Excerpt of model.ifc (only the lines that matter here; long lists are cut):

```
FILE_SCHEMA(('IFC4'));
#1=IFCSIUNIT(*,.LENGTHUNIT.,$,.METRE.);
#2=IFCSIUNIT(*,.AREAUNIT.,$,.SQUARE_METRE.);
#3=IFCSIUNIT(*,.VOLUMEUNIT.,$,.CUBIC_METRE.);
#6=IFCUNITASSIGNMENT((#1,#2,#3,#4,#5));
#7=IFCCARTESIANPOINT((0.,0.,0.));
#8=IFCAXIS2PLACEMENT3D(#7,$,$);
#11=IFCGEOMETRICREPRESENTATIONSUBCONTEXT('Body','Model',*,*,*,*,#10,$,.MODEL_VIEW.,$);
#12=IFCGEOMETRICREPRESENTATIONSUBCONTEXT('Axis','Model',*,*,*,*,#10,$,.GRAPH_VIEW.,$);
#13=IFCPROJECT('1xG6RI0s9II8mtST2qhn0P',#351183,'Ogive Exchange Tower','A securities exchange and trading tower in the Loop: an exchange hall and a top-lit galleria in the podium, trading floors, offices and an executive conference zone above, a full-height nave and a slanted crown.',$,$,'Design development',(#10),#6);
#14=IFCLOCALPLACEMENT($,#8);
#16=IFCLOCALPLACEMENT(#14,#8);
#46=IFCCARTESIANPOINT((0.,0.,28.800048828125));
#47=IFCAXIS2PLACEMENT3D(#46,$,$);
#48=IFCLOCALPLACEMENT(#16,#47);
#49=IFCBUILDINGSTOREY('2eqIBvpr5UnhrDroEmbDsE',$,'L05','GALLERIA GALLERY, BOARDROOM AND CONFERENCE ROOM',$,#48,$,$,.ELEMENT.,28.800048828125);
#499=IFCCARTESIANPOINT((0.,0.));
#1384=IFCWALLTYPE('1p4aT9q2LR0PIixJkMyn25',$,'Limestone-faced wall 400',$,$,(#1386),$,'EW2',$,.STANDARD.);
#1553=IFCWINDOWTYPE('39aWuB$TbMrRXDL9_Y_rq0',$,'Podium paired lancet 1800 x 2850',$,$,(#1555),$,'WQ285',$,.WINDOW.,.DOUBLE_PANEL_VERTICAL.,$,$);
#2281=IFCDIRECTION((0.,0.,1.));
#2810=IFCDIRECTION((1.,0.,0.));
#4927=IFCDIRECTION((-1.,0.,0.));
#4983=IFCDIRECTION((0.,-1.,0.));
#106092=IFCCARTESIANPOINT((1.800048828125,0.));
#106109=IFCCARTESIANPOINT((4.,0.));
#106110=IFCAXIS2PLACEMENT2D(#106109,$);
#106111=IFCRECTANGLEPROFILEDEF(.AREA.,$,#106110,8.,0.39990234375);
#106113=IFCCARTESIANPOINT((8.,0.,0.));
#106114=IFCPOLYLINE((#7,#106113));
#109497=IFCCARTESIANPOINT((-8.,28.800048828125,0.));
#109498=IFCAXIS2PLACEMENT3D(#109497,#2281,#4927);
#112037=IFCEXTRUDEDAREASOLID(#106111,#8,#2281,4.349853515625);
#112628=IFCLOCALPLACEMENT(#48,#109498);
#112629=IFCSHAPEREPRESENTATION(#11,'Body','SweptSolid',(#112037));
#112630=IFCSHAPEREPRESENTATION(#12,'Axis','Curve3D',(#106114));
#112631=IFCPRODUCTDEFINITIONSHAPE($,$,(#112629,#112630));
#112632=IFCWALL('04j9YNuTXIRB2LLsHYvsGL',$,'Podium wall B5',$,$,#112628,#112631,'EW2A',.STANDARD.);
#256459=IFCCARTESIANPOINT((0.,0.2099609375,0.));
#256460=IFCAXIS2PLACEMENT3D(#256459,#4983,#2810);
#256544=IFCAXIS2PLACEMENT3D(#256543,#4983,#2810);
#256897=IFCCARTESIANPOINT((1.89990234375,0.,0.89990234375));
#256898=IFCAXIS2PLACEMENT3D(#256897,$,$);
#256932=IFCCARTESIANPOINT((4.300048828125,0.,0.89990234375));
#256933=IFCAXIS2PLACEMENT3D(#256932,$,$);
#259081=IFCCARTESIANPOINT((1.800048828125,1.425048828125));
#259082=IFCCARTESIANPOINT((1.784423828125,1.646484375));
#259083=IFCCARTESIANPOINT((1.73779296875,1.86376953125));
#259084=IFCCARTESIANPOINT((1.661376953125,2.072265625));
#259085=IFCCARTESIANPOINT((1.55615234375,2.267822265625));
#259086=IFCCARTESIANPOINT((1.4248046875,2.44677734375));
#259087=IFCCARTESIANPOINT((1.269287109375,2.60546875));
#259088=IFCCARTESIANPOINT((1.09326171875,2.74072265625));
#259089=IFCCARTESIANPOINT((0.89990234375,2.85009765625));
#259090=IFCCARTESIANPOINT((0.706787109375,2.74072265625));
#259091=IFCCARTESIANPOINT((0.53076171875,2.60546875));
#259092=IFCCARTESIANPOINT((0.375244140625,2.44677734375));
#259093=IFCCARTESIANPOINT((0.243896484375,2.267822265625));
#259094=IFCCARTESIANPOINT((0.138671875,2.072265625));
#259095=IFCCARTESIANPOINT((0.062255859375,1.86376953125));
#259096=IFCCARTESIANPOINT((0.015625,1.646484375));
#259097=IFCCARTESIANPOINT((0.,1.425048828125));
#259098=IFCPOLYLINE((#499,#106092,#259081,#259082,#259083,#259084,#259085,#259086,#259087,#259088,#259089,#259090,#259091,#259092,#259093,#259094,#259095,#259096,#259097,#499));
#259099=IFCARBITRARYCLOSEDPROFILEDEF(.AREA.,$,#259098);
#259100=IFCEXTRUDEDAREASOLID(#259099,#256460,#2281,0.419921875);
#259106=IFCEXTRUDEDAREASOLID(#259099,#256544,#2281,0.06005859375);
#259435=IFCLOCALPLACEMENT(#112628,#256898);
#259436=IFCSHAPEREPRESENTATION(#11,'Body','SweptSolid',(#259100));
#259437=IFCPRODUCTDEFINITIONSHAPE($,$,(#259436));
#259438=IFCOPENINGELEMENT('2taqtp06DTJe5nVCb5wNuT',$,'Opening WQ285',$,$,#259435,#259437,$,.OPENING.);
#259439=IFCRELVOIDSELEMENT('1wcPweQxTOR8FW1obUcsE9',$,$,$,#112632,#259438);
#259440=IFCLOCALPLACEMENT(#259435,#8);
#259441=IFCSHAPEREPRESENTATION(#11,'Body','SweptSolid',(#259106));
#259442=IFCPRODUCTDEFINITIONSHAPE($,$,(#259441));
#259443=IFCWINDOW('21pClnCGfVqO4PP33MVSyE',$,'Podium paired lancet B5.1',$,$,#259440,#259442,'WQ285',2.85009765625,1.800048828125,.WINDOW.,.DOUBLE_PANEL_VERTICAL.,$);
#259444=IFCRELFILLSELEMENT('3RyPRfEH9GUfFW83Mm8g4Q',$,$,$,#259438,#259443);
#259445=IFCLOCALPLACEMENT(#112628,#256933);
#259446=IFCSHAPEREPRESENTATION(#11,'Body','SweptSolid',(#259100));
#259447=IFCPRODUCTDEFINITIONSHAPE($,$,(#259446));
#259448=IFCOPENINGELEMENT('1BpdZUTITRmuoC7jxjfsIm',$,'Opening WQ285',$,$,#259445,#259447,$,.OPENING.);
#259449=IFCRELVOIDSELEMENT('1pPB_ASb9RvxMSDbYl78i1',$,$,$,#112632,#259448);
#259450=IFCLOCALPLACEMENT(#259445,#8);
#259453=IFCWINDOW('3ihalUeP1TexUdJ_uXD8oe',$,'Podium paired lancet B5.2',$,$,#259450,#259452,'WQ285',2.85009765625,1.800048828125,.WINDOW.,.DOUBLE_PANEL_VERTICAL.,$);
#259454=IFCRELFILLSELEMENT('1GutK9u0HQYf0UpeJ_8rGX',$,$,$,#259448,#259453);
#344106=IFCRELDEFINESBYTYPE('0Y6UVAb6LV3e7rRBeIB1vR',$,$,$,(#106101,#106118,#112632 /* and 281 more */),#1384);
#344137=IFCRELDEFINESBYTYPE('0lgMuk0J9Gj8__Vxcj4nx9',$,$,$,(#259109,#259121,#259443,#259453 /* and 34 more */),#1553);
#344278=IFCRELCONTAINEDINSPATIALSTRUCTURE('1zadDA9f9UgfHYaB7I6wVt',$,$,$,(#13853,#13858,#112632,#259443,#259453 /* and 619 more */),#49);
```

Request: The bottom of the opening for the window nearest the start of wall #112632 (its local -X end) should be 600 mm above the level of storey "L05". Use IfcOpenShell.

```python
import numpy as np
import ifcopenshell
import ifcopenshell.api.geometry
import ifcopenshell.geom
import ifcopenshell.util.element
import ifcopenshell.util.placement
import ifcopenshell.util.shape
import ifcopenshell.util.unit

model = ifcopenshell.open("model.ifc")
unit_scale = ifcopenshell.util.unit.calculate_unit_scale(model)

window = model.by_guid("21pClnCGfVqO4PP33MVSyE")
opening = window.FillsVoids[0].RelatingOpeningElement
storey = ifcopenshell.util.element.get_container(window, ifc_class="IfcBuildingStorey")
level = ifcopenshell.util.placement.get_local_placement(storey.ObjectPlacement)[2, 3]

# The opening's origin need not be at the sill, so measure its lowest point.
shape = ifcopenshell.geom.create_shape(ifcopenshell.geom.settings(), opening)
bottom = ifcopenshell.util.shape.get_shape_bottom_elevation(shape, shape.geometry) / unit_scale
dz = level + 0.6 - bottom

shift = np.array([0.0, 0.0, dz])
# The window is placed relative to its opening, so it follows when the opening moves.
matrix = ifcopenshell.util.placement.get_local_placement(opening.ObjectPlacement)
matrix[:3, 3] += shift
ifcopenshell.api.geometry.edit_object_placement(
    model, product=opening, matrix=matrix, is_si=False, should_transform_children=True
)

print(f"moved by {dz * unit_scale:+.3f} m")

model.write("model_rev.ifc")
```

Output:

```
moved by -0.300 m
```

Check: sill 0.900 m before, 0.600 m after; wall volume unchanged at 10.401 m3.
